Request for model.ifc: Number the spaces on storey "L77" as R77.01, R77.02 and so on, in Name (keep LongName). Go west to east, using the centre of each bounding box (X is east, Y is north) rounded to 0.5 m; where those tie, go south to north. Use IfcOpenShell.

First a look at what the model holds.

```python
import ifcopenshell
import ifcopenshell.util.element
import ifcopenshell.util.placement

model = ifcopenshell.open("model.ifc")
print(model.schema)
storey = next(s for s in model.by_type("IfcBuildingStorey") if s.Name == "L77")
spaces = [e for e in ifcopenshell.util.element.get_decomposition(storey) if e.is_a("IfcSpace")]
for e in sorted(spaces, key=lambda e: e.id()):
    origin = ifcopenshell.util.placement.get_local_placement(e.ObjectPlacement)[:3, 3]
    print(e.id(), e.Name, e.LongName, origin.round(2) + 0.0, sep=" | ")
```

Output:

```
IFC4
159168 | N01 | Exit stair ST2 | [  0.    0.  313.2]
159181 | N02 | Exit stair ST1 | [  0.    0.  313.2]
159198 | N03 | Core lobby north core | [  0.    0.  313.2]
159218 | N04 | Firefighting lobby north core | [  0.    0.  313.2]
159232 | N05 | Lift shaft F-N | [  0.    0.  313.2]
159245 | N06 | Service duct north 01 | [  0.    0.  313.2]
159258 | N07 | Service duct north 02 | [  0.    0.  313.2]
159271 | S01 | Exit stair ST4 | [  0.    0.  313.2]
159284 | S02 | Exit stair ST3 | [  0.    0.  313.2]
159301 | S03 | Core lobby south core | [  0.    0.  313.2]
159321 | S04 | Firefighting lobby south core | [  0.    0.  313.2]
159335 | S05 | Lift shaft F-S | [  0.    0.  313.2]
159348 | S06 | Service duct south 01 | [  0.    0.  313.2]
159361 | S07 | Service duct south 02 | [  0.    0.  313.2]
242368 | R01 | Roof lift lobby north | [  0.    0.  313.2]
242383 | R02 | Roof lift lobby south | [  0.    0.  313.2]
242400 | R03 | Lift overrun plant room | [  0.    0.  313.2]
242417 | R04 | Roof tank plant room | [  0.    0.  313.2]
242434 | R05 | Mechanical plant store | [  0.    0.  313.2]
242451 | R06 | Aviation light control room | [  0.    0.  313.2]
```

```python
import ifcopenshell
import ifcopenshell.geom
import ifcopenshell.util.element
import ifcopenshell.util.shape

model = ifcopenshell.open("model.ifc")
settings = ifcopenshell.geom.settings()
settings.set("use-world-coords", True)


def centre(element):
    shape = ifcopenshell.geom.create_shape(settings, element)
    return ifcopenshell.util.shape.get_bbox_centroid(shape.geometry)


storey = next(s for s in model.by_type("IfcBuildingStorey") if s.Name == "L77")
spaces = [e for e in ifcopenshell.util.element.get_decomposition(storey) if e.is_a("IfcSpace")]

# Insertion points can sit at a corner or the storey origin, so sort by the geometry (in metres).
centres = {e: centre(e) for e in spaces}
spaces.sort(key=lambda e: (round(centres[e][0] / 0.5), centres[e][1]))

for i, e in enumerate(spaces, start=1):
    number = f"R77.{i:02d}"
    e.Name = number
    print(e.id(), number)

model.write("model_edited.ifc")
```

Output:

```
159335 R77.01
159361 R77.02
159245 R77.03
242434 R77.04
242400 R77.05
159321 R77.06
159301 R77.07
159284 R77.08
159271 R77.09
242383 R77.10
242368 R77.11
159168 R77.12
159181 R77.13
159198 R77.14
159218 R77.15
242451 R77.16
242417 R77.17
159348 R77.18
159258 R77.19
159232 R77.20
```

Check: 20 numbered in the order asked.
